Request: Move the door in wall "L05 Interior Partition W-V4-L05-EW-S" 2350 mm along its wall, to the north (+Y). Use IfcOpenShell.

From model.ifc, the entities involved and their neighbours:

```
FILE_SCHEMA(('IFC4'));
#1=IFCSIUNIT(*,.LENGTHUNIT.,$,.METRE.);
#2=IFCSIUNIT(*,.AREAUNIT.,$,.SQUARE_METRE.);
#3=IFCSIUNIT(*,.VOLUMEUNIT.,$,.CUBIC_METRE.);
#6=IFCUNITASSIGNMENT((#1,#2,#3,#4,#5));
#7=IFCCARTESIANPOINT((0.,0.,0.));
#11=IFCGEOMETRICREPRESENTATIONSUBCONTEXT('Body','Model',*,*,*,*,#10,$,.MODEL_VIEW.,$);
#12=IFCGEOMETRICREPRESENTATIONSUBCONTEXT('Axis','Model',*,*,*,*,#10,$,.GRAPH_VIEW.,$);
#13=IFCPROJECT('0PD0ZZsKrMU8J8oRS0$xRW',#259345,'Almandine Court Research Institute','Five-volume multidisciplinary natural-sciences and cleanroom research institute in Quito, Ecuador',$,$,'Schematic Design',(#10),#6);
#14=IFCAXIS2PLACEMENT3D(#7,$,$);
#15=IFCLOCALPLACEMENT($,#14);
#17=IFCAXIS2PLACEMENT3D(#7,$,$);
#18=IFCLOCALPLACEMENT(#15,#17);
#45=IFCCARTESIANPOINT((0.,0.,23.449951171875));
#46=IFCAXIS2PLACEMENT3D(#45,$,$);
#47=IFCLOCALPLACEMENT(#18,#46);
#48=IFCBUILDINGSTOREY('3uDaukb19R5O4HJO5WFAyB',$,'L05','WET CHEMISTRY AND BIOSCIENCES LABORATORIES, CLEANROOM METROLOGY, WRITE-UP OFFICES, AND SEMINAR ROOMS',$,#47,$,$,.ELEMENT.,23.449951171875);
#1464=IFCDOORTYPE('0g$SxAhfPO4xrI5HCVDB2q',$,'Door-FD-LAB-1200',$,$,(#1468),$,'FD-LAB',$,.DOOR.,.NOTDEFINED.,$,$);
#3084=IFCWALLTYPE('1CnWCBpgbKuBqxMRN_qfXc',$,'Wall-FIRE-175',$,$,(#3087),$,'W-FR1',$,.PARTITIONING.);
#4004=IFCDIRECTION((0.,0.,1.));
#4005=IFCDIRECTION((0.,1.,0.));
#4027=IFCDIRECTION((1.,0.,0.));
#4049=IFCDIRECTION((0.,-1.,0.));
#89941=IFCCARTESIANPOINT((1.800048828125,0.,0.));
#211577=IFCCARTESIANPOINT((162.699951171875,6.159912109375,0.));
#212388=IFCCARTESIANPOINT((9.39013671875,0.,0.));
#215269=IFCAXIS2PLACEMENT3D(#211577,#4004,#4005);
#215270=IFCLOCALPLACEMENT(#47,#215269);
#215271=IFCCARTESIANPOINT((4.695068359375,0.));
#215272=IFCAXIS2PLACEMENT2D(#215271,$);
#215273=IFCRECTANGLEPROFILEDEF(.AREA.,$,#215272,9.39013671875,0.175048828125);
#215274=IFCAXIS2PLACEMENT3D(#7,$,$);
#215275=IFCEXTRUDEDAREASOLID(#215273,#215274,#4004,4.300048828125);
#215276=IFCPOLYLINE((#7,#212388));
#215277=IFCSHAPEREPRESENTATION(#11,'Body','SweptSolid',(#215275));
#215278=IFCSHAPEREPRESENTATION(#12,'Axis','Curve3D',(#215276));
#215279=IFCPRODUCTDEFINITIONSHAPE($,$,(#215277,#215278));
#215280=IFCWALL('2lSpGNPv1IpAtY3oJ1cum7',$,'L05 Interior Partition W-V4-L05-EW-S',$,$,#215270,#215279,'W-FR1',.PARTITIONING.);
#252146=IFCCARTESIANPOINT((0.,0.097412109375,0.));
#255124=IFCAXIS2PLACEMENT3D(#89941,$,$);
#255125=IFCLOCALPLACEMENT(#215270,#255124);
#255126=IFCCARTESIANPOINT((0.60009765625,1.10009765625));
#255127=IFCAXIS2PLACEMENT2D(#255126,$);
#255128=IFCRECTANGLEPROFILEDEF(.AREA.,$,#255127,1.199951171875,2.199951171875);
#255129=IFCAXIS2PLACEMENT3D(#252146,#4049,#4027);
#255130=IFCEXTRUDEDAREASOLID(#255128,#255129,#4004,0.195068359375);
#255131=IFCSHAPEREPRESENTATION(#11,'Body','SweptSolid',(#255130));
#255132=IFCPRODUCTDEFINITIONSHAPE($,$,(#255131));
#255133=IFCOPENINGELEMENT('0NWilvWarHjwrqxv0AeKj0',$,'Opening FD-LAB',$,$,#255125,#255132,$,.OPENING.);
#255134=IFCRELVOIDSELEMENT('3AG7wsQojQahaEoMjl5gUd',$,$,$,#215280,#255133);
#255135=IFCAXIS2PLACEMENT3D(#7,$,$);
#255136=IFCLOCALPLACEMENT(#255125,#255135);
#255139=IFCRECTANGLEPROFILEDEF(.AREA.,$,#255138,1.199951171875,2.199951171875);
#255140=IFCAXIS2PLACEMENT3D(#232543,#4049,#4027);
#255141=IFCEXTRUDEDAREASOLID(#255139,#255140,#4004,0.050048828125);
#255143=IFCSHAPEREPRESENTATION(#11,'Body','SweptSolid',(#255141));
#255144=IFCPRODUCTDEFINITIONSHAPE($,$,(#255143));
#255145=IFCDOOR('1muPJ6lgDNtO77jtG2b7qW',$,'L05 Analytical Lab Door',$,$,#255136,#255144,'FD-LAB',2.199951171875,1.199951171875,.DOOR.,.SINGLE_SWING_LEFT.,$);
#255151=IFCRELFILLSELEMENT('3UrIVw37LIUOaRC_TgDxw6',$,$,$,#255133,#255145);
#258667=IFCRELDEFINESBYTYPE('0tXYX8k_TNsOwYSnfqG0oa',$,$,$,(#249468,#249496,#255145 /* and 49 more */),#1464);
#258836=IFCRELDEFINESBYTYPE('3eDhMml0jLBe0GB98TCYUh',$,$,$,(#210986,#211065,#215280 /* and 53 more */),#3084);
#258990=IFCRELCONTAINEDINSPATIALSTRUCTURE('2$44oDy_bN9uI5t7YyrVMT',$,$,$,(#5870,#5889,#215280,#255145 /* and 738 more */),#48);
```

```python
import ifcopenshell
import ifcopenshell.api.geometry
import ifcopenshell.util.placement
import ifcopenshell.util.unit

model = ifcopenshell.open("model.ifc")
unit_scale = ifcopenshell.util.unit.calculate_unit_scale(model)

door = model.by_guid("1muPJ6lgDNtO77jtG2b7qW")
opening = door.FillsVoids[0].RelatingOpeningElement
wall = opening.VoidsElements[0].RelatingBuildingElement

wall_matrix = ifcopenshell.util.placement.get_local_placement(wall.ObjectPlacement)
shift = wall_matrix[:3, 0] * 2.35 / unit_scale
before = ifcopenshell.util.placement.get_local_placement(door.ObjectPlacement)[:3, 3].copy()

# The door is placed relative to its opening, so it follows when the opening moves.
matrix = ifcopenshell.util.placement.get_local_placement(opening.ObjectPlacement)
matrix[:3, 3] += shift
ifcopenshell.api.geometry.edit_object_placement(
    model, product=opening, matrix=matrix, is_si=False, should_transform_children=True
)

after = ifcopenshell.util.placement.get_local_placement(door.ObjectPlacement)[:3, 3]
print("door moved by", (after - before).round(3) + 0.0)

model.write("model_edited.ifc")
```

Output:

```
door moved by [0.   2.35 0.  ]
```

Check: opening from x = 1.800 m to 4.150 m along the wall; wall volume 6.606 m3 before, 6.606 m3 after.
